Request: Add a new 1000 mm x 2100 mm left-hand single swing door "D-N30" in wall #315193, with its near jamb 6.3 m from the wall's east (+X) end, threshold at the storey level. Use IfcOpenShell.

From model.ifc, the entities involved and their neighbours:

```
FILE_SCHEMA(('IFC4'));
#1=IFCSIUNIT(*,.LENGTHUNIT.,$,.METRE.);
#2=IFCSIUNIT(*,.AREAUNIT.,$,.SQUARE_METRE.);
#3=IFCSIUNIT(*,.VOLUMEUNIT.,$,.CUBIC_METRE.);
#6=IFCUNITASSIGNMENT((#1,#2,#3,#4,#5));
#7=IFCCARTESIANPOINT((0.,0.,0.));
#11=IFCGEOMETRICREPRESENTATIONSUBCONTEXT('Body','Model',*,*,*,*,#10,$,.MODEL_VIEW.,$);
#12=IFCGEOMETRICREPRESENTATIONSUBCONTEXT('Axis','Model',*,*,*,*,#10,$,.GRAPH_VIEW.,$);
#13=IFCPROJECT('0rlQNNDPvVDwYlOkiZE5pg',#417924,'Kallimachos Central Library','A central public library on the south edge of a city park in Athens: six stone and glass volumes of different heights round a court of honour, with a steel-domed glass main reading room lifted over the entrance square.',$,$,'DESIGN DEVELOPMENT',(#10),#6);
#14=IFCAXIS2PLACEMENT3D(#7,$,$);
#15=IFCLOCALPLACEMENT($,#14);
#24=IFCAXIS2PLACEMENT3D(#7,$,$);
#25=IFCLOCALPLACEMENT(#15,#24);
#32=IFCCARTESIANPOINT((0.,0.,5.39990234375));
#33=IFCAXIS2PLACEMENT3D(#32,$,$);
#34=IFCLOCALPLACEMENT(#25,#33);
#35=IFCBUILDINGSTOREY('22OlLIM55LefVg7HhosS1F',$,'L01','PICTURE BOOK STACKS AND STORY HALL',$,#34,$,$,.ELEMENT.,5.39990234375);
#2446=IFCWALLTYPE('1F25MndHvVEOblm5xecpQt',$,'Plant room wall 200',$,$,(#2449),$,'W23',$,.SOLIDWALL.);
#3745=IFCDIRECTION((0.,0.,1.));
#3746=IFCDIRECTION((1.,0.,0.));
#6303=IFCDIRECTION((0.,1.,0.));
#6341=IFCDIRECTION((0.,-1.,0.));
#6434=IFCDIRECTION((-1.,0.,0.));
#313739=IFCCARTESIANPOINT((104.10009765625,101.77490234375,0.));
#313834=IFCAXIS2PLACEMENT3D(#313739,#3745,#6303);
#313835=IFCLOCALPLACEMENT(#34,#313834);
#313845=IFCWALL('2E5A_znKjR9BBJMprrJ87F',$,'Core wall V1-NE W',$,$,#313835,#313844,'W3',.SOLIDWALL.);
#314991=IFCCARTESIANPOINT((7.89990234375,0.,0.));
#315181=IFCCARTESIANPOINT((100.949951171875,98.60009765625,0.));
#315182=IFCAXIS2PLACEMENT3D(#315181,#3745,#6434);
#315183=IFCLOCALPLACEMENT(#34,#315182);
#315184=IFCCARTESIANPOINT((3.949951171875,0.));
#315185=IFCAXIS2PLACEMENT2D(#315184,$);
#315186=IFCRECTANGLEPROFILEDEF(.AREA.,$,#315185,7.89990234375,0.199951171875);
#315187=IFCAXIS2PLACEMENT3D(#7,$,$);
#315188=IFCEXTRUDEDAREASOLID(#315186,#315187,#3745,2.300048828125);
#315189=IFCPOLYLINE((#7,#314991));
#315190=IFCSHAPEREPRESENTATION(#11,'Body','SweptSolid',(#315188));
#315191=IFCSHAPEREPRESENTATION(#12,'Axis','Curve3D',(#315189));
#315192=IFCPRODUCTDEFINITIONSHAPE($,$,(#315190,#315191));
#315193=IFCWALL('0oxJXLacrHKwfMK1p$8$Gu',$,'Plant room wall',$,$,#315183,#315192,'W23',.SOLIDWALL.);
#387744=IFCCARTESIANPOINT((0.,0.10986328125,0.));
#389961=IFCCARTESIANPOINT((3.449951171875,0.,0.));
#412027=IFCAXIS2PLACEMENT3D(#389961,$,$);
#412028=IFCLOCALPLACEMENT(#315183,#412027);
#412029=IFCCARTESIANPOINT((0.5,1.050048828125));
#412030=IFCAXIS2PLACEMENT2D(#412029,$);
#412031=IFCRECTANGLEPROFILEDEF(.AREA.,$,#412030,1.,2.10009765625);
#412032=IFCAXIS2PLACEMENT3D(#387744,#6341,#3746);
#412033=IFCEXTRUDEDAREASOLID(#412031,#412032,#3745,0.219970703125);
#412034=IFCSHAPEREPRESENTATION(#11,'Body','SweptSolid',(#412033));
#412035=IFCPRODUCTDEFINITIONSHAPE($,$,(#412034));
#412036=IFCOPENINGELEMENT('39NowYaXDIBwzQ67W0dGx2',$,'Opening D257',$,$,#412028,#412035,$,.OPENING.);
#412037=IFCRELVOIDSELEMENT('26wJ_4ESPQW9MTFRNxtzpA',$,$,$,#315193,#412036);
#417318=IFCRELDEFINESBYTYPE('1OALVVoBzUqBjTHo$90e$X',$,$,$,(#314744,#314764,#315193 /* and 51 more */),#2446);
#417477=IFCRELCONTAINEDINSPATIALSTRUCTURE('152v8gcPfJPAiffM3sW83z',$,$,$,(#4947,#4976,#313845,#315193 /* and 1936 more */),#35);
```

```python
import numpy as np
import ifcopenshell
import ifcopenshell.api.feature
import ifcopenshell.api.geometry
import ifcopenshell.api.root
import ifcopenshell.api.spatial
import ifcopenshell.geom
import ifcopenshell.util.element
import ifcopenshell.util.placement
import ifcopenshell.util.representation
import ifcopenshell.util.shape
import ifcopenshell.util.unit

model = ifcopenshell.open("model.ifc")
unit_scale = ifcopenshell.util.unit.calculate_unit_scale(model)
settings = ifcopenshell.geom.settings()


def volume(element):
    """Net volume in cubic metres, openings subtracted."""
    shape = ifcopenshell.geom.create_shape(settings, element)
    return ifcopenshell.util.shape.get_volume(shape.geometry)


wall = model.by_id(315193)
storey = ifcopenshell.util.element.get_container(wall, ifc_class="IfcBuildingStorey")
context = ifcopenshell.util.representation.get_context(model, "Model", "Body", "MODEL_VIEW")
before = volume(wall)

width, height, from_end, sill = 1, 2.1, 6.3, 0.0  # metres

# The wall runs along its own X axis, and the end named is its -X end.
wall_shape = ifcopenshell.geom.create_shape(settings, wall)
x, y, z = ifcopenshell.util.shape.get_vertices(wall_shape.geometry).T
start = x.min() + from_end
face, thickness = float(y.min()), float(y.max() - y.min())
wall_matrix = ifcopenshell.util.placement.get_local_placement(wall.ObjectPlacement)
level = ifcopenshell.util.placement.get_local_placement(storey.ObjectPlacement)[2, 3]


def in_wall(x, y):
    """Placement at x, y metres in the wall's axes, at sill height."""
    matrix = wall_matrix.copy()
    matrix[:, 3] = wall_matrix @ np.array([x / unit_scale, y / unit_scale, 0.0, 1.0])
    matrix[2, 3] = level + sill / unit_scale
    return matrix


# Opening: a box that overshoots both wall faces by 50 mm.
opening = ifcopenshell.api.root.create_entity(model, ifc_class="IfcOpeningElement", predefined_type="OPENING")
box = ifcopenshell.api.geometry.add_wall_representation(
    model, context=context, length=width, height=height, thickness=thickness + 0.1
)
ifcopenshell.api.geometry.assign_representation(model, product=opening, representation=box)
ifcopenshell.api.geometry.edit_object_placement(model, product=opening, matrix=in_wall(start, face - 0.05), is_si=False)
ifcopenshell.api.feature.add_feature(model, feature=opening, element=wall)

door = ifcopenshell.api.root.create_entity(model, ifc_class="IfcDoor", name="D-N30", predefined_type="DOOR")
door.OverallWidth, door.OverallHeight = width / unit_scale, height / unit_scale
door.OperationType = "SINGLE_SWING_LEFT"
body = ifcopenshell.api.geometry.add_door_representation(
    model,
    context=context,
    overall_width=door.OverallWidth,
    overall_height=door.OverallHeight,
    operation_type="SINGLE_SWING_LEFT",
    lining_properties={"LiningDepth": thickness / unit_scale, "ThresholdDepth": thickness / unit_scale},
)
ifcopenshell.api.geometry.assign_representation(model, product=door, representation=body)
ifcopenshell.api.spatial.assign_container(model, products=[door], relating_structure=storey)
ifcopenshell.api.feature.add_filling(model, opening=opening, element=door)

# The lining spans the wall, so the door starts at the wall face.
ifcopenshell.api.geometry.edit_object_placement(model, product=door, matrix=in_wall(start, face), is_si=False)

after = volume(wall)

print(f"wall volume {before:.3f} -> {after:.3f} m3")

model.write("model_v2.ifc")
```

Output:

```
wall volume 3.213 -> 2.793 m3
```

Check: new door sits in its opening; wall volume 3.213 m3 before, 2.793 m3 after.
